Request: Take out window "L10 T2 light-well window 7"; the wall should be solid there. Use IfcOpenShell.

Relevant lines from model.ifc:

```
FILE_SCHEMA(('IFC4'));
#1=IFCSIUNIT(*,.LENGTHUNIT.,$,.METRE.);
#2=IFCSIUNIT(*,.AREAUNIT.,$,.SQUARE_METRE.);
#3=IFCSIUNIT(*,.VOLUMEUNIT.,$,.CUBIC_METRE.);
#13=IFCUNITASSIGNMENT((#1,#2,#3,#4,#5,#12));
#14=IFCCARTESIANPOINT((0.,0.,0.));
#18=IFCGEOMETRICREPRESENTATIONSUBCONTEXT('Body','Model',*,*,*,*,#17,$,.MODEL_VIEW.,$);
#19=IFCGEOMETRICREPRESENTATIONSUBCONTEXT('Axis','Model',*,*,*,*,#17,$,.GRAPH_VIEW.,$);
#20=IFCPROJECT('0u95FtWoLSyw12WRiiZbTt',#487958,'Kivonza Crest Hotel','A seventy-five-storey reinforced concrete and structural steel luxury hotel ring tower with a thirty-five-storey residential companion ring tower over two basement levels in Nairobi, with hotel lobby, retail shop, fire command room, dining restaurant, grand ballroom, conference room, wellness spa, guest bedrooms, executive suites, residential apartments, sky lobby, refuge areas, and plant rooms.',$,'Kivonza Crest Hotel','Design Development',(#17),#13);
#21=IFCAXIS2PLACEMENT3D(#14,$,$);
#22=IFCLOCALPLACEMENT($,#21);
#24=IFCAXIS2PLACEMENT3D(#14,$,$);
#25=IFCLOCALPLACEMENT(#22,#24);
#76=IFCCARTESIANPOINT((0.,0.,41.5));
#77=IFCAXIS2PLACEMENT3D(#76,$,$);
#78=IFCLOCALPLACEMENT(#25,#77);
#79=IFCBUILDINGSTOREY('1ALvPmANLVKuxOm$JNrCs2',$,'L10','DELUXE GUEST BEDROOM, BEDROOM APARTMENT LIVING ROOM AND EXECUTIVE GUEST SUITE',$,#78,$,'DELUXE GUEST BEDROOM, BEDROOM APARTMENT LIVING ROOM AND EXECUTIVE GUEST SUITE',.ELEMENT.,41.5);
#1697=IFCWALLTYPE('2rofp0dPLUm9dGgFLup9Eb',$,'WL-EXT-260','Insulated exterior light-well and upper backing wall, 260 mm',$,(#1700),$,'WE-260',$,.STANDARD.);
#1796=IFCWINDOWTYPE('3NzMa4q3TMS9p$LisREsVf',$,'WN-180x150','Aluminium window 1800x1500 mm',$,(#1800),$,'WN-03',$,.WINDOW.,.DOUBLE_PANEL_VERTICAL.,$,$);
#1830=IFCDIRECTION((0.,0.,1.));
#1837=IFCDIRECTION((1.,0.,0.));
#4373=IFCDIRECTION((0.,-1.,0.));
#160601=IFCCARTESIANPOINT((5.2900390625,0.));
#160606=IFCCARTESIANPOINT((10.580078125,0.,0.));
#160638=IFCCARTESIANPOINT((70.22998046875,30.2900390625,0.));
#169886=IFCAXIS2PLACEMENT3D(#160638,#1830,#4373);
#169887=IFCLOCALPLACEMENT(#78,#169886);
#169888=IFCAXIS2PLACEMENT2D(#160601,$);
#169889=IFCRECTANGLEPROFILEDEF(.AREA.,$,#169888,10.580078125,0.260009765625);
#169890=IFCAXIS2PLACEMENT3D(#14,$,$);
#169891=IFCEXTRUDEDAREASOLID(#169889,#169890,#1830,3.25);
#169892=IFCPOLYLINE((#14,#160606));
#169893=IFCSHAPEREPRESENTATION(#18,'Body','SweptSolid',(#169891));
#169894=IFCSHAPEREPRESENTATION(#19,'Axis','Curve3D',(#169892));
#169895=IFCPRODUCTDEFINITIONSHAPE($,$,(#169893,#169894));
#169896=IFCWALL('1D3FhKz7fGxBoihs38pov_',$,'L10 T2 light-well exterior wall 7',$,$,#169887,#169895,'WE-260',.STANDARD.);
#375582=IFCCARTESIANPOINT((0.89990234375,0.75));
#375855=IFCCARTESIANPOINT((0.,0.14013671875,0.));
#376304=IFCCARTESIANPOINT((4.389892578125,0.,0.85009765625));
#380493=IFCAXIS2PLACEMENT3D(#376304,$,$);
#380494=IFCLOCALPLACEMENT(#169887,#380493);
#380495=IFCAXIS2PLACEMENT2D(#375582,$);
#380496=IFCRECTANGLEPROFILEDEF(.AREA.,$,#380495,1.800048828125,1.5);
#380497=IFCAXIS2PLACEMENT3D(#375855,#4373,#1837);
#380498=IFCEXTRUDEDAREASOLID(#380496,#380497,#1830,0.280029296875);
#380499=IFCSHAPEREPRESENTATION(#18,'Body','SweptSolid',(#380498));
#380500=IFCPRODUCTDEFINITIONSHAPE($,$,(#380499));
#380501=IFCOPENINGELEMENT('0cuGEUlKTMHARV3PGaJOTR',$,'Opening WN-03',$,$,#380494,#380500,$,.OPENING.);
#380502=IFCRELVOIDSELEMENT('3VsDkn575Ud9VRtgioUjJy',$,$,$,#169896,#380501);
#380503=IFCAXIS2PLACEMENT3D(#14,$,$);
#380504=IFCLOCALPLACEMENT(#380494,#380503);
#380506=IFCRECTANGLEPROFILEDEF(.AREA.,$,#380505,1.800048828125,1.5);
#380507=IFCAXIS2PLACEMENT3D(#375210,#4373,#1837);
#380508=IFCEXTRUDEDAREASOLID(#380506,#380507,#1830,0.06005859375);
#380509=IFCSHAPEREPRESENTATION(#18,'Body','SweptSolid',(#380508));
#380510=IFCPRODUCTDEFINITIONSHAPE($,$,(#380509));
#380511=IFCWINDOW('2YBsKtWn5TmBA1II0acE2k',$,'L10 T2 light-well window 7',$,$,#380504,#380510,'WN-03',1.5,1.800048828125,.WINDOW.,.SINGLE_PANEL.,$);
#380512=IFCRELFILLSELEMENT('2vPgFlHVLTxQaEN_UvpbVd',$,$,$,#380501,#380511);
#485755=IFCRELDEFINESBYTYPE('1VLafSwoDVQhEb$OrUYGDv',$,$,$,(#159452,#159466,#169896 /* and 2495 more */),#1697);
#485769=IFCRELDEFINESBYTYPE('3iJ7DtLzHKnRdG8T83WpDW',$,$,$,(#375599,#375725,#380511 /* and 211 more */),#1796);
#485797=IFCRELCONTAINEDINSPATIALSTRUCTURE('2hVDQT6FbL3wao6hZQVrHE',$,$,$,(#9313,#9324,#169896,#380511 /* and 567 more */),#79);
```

```python
import ifcopenshell
import ifcopenshell.api.feature
import ifcopenshell.api.root
import ifcopenshell.geom
import ifcopenshell.util.shape

model = ifcopenshell.open("model.ifc")
settings = ifcopenshell.geom.settings()


def volume(element):
    """Net volume in cubic metres, openings subtracted."""
    shape = ifcopenshell.geom.create_shape(settings, element)
    return ifcopenshell.util.shape.get_volume(shape.geometry)


window = model.by_guid("2YBsKtWn5TmBA1II0acE2k")
opening = window.FillsVoids[0].RelatingOpeningElement
wall = opening.VoidsElements[0].RelatingBuildingElement
before = volume(wall)

ifcopenshell.api.root.remove_product(model, product=window)
ifcopenshell.api.feature.remove_feature(model, feature=opening)

after = volume(wall)

print(f"wall volume {before:.3f} -> {after:.3f} m3")

model.write("model-out.ifc")
```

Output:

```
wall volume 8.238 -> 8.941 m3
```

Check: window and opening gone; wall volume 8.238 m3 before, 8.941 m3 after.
